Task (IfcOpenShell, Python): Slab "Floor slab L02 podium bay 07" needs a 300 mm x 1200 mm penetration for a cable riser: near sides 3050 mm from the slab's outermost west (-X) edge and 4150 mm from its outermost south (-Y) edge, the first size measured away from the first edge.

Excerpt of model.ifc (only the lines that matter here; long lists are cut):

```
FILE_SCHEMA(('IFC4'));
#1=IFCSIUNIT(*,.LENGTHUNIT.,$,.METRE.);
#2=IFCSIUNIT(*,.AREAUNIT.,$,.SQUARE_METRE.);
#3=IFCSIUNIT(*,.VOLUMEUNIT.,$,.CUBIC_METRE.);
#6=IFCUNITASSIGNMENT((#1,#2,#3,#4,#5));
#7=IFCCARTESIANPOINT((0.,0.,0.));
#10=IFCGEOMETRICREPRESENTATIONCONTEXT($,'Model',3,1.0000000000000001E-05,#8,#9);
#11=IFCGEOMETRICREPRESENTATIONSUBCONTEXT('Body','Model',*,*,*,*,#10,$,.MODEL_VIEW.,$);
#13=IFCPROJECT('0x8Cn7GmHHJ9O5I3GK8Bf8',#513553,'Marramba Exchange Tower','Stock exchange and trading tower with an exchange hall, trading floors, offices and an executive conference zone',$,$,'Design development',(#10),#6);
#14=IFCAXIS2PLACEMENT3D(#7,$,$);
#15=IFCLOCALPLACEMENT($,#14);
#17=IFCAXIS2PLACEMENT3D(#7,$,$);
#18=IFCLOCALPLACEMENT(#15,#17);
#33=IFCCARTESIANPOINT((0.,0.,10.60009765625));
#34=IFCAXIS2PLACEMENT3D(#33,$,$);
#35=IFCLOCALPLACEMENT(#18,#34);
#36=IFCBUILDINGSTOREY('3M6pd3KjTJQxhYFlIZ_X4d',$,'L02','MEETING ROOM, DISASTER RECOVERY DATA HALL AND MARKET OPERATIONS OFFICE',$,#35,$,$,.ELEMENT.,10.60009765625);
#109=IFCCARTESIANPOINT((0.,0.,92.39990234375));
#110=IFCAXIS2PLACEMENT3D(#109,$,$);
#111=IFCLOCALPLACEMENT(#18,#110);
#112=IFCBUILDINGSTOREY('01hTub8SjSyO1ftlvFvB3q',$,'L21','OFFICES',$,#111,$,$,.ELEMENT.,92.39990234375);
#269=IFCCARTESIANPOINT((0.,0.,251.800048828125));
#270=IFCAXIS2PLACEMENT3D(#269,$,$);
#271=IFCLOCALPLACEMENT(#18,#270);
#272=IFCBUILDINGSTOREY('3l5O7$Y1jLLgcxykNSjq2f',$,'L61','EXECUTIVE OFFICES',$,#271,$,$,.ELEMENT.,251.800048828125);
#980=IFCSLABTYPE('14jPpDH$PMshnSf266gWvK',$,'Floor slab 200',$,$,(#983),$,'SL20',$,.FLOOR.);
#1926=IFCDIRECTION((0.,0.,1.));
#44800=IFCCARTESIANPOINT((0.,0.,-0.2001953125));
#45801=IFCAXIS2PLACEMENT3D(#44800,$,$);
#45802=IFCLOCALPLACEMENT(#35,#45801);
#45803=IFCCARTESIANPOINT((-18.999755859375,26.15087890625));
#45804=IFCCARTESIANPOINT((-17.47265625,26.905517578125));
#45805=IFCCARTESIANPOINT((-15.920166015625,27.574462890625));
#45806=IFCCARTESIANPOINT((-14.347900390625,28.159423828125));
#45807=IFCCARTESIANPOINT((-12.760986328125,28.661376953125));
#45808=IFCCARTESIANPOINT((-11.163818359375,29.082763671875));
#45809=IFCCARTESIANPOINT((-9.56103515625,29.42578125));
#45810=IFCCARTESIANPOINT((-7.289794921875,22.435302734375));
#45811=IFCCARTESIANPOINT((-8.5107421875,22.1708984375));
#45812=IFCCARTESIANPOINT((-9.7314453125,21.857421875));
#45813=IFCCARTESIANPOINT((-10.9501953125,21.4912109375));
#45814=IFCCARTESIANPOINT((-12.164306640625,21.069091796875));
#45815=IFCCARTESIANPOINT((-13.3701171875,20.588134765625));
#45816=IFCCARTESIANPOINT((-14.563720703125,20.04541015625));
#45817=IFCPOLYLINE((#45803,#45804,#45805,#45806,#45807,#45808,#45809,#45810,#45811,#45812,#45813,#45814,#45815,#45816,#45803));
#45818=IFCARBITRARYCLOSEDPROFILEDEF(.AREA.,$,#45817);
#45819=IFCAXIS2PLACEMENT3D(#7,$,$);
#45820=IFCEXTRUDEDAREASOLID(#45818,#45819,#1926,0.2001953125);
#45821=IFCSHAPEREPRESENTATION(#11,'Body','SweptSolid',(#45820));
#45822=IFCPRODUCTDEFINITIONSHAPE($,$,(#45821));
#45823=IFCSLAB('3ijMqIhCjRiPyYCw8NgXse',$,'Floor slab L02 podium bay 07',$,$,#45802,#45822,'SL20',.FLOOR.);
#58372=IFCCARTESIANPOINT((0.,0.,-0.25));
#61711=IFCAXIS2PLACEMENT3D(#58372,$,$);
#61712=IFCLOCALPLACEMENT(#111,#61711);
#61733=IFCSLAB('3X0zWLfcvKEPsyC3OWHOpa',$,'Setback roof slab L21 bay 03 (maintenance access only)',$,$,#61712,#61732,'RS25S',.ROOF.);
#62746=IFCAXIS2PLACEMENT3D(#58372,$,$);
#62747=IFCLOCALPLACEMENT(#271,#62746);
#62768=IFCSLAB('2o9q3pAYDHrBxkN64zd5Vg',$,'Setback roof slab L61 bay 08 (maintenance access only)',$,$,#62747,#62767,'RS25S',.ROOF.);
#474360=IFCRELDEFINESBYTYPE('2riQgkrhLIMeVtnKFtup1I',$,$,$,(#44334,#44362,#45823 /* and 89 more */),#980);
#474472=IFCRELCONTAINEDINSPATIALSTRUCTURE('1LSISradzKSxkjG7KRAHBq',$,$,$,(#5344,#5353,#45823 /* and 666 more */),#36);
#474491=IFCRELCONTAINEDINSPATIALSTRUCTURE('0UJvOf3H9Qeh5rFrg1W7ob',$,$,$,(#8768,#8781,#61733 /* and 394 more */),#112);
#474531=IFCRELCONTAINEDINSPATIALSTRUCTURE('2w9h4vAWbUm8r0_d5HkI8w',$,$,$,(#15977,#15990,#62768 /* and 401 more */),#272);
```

```python
import numpy as np
import ifcopenshell
import ifcopenshell.api.feature
import ifcopenshell.api.geometry
import ifcopenshell.api.root
import ifcopenshell.geom
import ifcopenshell.util.placement
import ifcopenshell.util.representation
import ifcopenshell.util.shape
import ifcopenshell.util.unit

model = ifcopenshell.open("model.ifc")
unit_scale = ifcopenshell.util.unit.calculate_unit_scale(model)
settings = ifcopenshell.geom.settings()


def volume(element):
    """Net volume in cubic metres, openings subtracted."""
    shape = ifcopenshell.geom.create_shape(settings, element)
    return ifcopenshell.util.shape.get_volume(shape.geometry)


slab = model.by_guid("3ijMqIhCjRiPyYCw8NgXse")
before = volume(slab)

# Extent in the slab's own axes, in metres. The edges named are its -X and -Y sides.
slab_shape = ifcopenshell.geom.create_shape(settings, slab)
vertices = ifcopenshell.util.shape.get_vertices(slab_shape.geometry)
x_min, y_min, bottom = vertices.min(axis=0)
top = vertices[:, 2].max()

opening = ifcopenshell.api.root.create_entity(model, ifc_class="IfcOpeningElement", name="Cable riser opening", predefined_type="OPENING")
context = ifcopenshell.util.representation.get_context(model, "Model", "Body", "MODEL_VIEW")
width, depth = 0.3, 1.2
outline = [(0.0, 0.0), (width, 0.0), (width, depth), (0.0, depth), (0.0, 0.0)]
# Overshoot both faces by 50 mm so the cut is clean.
shape = ifcopenshell.api.geometry.add_slab_representation(
    model, context=context, depth=top - bottom + 0.1, polyline=outline
)
ifcopenshell.api.geometry.assign_representation(model, product=opening, representation=shape)

matrix = ifcopenshell.util.placement.get_local_placement(slab.ObjectPlacement)
matrix[:, 3] = matrix @ np.append(np.array([x_min + 3.05, y_min + 4.15, bottom - 0.05]) / unit_scale, 1.0)
ifcopenshell.api.geometry.edit_object_placement(model, product=opening, matrix=matrix, is_si=False)
ifcopenshell.api.feature.add_feature(model, feature=opening, element=slab)

after = volume(slab)

print(f"slab volume {before:.3f} -> {after:.3f} m3")

model.write("model_v2.ifc")
```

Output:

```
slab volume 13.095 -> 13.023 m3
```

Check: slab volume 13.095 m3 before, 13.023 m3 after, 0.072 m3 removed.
